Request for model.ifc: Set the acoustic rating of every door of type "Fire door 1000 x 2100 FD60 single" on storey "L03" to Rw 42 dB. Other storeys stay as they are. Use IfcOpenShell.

First a look at what the model holds.

```python
import ifcopenshell
import ifcopenshell.util.element

model = ifcopenshell.open("model.ifc")
print(model.schema)
storey = next(s for s in model.by_type("IfcBuildingStorey") if s.Name == "L03")
doors = [e for e in ifcopenshell.util.element.get_decomposition(storey) if e.is_a("IfcDoor")]
seen = {}
for e in doors:
    element_type = ifcopenshell.util.element.get_type(e)
    key = (element_type.Name if element_type != e and element_type else None, ifcopenshell.util.element.get_pset(e, "Pset_DoorCommon", "AcousticRating"))
    seen[key] = seen.get(key, 0) + 1
for (name, value), count in sorted(seen.items(), key=str):
    print(count, "x", name, "|", value)
```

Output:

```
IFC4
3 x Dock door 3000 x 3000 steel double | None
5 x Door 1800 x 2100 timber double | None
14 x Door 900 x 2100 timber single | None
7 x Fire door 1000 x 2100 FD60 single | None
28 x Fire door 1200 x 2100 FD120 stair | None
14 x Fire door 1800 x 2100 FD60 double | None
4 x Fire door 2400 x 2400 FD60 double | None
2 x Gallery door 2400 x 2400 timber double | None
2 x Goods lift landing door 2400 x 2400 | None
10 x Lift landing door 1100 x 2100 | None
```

```python
import ifcopenshell
import ifcopenshell.api.pset
import ifcopenshell.util.element

model = ifcopenshell.open("model.ifc")

storey = next(s for s in model.by_type("IfcBuildingStorey") if s.Name == "L03")
doors = [e for e in ifcopenshell.util.element.get_decomposition(storey) if e.is_a("IfcDoor")]

count = 0
for e in doors:
    element_type = ifcopenshell.util.element.get_type(e)
    if element_type in (None, e) or element_type.Name != "Fire door 1000 x 2100 FD60 single":
        continue
    # add_pset returns the element's existing set when there is one.
    pset = ifcopenshell.api.pset.add_pset(model, product=e, name="Pset_DoorCommon")
    ifcopenshell.api.pset.edit_pset(model, pset=pset, properties={"AcousticRating": "Rw 42 dB"})
    count += 1

print(count, "doors updated")

model.write("model_v2.ifc")
```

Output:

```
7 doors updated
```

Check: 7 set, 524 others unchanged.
